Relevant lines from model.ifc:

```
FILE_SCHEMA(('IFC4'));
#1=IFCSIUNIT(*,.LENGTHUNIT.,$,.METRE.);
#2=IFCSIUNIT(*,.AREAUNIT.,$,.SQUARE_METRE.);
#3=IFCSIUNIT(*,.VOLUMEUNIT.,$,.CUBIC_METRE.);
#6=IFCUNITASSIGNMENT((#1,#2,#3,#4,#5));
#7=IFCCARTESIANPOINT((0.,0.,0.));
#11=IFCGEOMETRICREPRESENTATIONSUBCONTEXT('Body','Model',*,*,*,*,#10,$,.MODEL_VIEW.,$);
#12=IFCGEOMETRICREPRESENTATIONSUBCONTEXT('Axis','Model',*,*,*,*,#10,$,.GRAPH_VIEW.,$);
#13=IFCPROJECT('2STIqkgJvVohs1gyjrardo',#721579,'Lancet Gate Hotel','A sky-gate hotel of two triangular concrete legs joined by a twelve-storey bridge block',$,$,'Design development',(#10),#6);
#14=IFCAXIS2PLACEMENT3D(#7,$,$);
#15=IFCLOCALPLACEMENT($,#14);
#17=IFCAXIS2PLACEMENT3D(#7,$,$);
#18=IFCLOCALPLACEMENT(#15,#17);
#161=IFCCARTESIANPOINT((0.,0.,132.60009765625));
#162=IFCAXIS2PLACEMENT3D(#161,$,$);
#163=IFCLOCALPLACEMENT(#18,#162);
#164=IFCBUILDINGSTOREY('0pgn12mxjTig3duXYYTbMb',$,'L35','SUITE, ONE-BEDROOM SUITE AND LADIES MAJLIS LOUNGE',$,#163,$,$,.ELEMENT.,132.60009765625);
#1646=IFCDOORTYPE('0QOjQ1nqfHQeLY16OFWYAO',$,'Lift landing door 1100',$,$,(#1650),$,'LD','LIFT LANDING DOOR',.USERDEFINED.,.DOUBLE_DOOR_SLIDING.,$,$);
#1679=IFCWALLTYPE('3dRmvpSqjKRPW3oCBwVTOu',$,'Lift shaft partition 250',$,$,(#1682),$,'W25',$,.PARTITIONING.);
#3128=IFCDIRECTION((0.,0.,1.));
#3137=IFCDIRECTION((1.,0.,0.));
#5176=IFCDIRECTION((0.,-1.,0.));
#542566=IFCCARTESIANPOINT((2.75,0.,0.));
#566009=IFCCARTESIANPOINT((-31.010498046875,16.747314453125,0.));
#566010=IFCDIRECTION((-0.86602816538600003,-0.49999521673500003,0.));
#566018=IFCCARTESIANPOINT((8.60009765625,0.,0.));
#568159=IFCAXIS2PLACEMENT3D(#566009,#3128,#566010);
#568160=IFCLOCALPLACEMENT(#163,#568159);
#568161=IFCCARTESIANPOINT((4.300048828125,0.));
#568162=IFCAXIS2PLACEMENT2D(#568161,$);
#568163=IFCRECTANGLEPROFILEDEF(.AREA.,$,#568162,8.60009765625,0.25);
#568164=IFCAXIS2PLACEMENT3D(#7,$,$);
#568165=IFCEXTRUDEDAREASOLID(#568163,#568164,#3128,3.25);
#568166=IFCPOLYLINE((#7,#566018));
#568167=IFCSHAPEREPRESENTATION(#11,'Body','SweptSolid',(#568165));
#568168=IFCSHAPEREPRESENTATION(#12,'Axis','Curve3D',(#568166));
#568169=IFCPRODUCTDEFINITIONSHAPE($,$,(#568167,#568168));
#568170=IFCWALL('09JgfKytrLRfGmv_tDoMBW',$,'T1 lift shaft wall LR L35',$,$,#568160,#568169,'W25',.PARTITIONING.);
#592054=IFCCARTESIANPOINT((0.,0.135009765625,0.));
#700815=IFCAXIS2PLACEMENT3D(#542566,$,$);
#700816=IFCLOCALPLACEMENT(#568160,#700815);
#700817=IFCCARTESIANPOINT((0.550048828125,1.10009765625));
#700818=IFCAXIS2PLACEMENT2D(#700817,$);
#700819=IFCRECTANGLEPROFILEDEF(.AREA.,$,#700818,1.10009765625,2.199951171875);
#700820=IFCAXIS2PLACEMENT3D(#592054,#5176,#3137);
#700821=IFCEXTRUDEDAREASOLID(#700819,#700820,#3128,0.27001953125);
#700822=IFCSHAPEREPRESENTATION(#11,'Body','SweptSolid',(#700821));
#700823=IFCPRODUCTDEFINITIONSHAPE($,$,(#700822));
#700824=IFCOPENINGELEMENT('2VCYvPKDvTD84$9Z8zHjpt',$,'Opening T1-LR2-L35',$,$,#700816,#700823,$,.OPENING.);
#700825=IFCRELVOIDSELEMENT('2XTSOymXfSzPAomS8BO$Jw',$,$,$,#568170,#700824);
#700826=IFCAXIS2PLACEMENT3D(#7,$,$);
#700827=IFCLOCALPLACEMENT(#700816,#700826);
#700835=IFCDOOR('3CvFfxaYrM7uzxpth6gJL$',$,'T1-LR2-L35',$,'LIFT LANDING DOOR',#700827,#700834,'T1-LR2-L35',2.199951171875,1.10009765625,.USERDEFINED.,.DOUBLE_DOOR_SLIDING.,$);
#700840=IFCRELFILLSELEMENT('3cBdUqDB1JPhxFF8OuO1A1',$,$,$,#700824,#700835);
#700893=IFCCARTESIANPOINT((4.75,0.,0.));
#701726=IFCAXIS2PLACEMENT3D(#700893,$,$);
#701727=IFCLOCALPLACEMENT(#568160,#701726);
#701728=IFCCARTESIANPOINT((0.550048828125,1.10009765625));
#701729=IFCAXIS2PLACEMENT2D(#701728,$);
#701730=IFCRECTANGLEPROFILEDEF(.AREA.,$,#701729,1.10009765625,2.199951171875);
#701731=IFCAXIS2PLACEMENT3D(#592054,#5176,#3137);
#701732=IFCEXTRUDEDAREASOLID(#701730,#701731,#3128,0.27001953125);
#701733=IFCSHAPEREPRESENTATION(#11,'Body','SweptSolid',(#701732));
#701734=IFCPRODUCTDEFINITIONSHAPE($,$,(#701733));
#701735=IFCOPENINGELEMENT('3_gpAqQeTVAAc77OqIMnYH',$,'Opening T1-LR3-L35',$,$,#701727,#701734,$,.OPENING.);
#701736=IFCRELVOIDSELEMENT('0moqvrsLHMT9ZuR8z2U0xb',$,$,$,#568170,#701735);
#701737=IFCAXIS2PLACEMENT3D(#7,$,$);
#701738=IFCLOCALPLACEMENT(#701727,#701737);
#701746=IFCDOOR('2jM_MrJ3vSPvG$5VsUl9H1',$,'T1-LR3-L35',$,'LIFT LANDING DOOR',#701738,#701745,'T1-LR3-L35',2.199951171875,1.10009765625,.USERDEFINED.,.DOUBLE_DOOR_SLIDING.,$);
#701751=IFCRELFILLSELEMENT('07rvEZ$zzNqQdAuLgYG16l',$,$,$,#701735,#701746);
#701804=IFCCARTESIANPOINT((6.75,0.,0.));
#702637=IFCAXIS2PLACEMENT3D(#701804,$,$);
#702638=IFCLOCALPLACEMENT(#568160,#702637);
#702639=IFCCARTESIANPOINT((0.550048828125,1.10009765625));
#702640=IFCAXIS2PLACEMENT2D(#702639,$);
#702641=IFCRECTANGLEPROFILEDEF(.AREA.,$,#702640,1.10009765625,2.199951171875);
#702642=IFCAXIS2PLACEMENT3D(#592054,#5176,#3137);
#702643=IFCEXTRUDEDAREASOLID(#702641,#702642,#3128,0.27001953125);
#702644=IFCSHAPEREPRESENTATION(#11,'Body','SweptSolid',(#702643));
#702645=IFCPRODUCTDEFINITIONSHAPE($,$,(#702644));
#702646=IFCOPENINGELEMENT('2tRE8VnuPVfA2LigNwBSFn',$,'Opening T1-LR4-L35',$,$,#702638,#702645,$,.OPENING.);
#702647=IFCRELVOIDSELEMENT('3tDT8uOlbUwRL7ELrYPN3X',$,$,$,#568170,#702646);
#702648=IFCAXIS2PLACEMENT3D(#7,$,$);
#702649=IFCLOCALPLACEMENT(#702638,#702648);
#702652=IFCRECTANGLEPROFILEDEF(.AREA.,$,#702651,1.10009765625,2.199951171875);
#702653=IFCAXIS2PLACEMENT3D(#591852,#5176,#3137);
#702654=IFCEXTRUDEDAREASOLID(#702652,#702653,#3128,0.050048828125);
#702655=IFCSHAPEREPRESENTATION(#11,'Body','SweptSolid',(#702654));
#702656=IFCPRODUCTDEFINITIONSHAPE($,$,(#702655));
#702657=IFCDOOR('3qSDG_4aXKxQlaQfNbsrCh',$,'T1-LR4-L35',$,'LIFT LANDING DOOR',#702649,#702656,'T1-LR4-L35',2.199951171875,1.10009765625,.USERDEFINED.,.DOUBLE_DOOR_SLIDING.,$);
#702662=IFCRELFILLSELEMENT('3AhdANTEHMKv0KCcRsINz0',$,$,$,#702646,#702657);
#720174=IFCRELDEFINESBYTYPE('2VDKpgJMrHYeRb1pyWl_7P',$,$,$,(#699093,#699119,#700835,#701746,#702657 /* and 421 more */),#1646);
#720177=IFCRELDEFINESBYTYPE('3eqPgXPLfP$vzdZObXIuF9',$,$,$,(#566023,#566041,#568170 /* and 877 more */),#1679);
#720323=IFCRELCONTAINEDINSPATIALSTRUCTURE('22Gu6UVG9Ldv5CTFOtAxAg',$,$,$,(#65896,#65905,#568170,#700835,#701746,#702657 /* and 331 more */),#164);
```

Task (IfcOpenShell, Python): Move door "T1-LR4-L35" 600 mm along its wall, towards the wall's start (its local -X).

```python
import ifcopenshell
import ifcopenshell.api.geometry
import ifcopenshell.util.placement
import ifcopenshell.util.unit

model = ifcopenshell.open("model.ifc")
unit_scale = ifcopenshell.util.unit.calculate_unit_scale(model)

door = model.by_guid("3qSDG_4aXKxQlaQfNbsrCh")
opening = door.FillsVoids[0].RelatingOpeningElement
wall = opening.VoidsElements[0].RelatingBuildingElement

wall_matrix = ifcopenshell.util.placement.get_local_placement(wall.ObjectPlacement)
shift = wall_matrix[:3, 0] * -0.6 / unit_scale
before = ifcopenshell.util.placement.get_local_placement(door.ObjectPlacement)[:3, 3].copy()

# The door is placed relative to its opening, so it follows when the opening moves.
matrix = ifcopenshell.util.placement.get_local_placement(opening.ObjectPlacement)
matrix[:3, 3] += shift
ifcopenshell.api.geometry.edit_object_placement(
    model, product=opening, matrix=matrix, is_si=False, should_transform_children=True
)

after = ifcopenshell.util.placement.get_local_placement(door.ObjectPlacement)[:3, 3]
print("door moved by", (after - before).round(3) + 0.0)

model.write("model_rev.ifc")
```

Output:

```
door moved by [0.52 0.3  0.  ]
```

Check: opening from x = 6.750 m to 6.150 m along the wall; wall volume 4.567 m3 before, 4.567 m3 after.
